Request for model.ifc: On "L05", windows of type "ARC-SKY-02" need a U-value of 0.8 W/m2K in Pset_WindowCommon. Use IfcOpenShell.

First a look at what the model holds.

```python
import ifcopenshell
import ifcopenshell.util.element

model = ifcopenshell.open("model.ifc")
print(model.schema)
storey = next(s for s in model.by_type("IfcBuildingStorey") if s.Name == "L05")
windows = [e for e in ifcopenshell.util.element.get_decomposition(storey) if e.is_a("IfcWindow")]
seen = {}
for e in windows:
    element_type = ifcopenshell.util.element.get_type(e)
    key = (element_type.Name if element_type != e and element_type else None, ifcopenshell.util.element.get_pset(e, "Pset_WindowCommon", "ThermalTransmittance"))
    seen[key] = seen.get(key, 0) + 1
for (name, value), count in sorted(seen.items(), key=str):
    print(count, "x", name, "|", value)
```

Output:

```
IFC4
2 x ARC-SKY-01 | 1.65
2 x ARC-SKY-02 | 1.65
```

```python
import ifcopenshell
import ifcopenshell.api.pset
import ifcopenshell.util.element

model = ifcopenshell.open("model.ifc")

storey = next(s for s in model.by_type("IfcBuildingStorey") if s.Name == "L05")
windows = [e for e in ifcopenshell.util.element.get_decomposition(storey) if e.is_a("IfcWindow")]

count = 0
for e in windows:
    element_type = ifcopenshell.util.element.get_type(e)
    if element_type in (None, e) or element_type.Name != "ARC-SKY-02":
        continue
    # add_pset returns the element's existing set when there is one.
    pset = ifcopenshell.api.pset.add_pset(model, product=e, name="Pset_WindowCommon")
    ifcopenshell.api.pset.edit_pset(model, pset=pset, properties={"ThermalTransmittance": 0.8})
    count += 1

print(count, "windows updated")

model.write("model_updated.ifc")
```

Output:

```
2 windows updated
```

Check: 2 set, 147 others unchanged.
